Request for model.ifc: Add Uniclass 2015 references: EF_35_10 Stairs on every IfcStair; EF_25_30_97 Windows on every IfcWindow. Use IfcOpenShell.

First a look at what the model holds.

```python
import ifcopenshell

model = ifcopenshell.open("model.ifc")
print(model.schema)
print("classifications:", [c.Name for c in model.by_type("IfcClassification")])
for ifc_class in ("IfcDoor", "IfcRoof", "IfcStair", "IfcWall", "IfcWindow"):
    print(ifc_class, len(model.by_type(ifc_class)))
```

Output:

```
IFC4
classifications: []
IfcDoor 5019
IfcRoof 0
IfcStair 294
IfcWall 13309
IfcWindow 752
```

```python
import ifcopenshell
import ifcopenshell.api.classification

model = ifcopenshell.open("model.ifc")

system = ifcopenshell.api.classification.add_classification(model, classification="Uniclass 2015")

codes = {
    "IfcStair": ("EF_35_10", "Stairs"),
    "IfcWindow": ("EF_25_30_97", "Windows"),
}
for ifc_class, (code, name) in codes.items():
    products = model.by_type(ifc_class)
    ifcopenshell.api.classification.add_reference(
        model, products=products, classification=system, identification=code, name=name
    )
    print(code, len(products))

model.write("model_edited.ifc")
```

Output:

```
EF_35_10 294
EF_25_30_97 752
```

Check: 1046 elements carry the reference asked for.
